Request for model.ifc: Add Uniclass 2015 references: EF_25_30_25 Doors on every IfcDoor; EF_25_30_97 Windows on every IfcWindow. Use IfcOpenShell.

First a look at what the model holds.

```python
import ifcopenshell

model = ifcopenshell.open("model.ifc")
print(model.schema)
print("classifications:", [c.Name for c in model.by_type("IfcClassification")])
for ifc_class in ("IfcDoor", "IfcRoof", "IfcStair", "IfcWall", "IfcWindow"):
    print(ifc_class, len(model.by_type(ifc_class)))
```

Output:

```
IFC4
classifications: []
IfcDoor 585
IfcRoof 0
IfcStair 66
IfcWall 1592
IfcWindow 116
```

```python
import ifcopenshell
import ifcopenshell.api.classification

model = ifcopenshell.open("model.ifc")

system = ifcopenshell.api.classification.add_classification(model, classification="Uniclass 2015")

codes = {
    "IfcDoor": ("EF_25_30_25", "Doors"),
    "IfcWindow": ("EF_25_30_97", "Windows"),
}
for ifc_class, (code, name) in codes.items():
    products = model.by_type(ifc_class)
    ifcopenshell.api.classification.add_reference(
        model, products=products, classification=system, identification=code, name=name
    )
    print(code, len(products))

model.write("model_v2.ifc")
```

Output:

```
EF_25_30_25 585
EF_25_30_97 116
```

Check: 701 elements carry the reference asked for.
